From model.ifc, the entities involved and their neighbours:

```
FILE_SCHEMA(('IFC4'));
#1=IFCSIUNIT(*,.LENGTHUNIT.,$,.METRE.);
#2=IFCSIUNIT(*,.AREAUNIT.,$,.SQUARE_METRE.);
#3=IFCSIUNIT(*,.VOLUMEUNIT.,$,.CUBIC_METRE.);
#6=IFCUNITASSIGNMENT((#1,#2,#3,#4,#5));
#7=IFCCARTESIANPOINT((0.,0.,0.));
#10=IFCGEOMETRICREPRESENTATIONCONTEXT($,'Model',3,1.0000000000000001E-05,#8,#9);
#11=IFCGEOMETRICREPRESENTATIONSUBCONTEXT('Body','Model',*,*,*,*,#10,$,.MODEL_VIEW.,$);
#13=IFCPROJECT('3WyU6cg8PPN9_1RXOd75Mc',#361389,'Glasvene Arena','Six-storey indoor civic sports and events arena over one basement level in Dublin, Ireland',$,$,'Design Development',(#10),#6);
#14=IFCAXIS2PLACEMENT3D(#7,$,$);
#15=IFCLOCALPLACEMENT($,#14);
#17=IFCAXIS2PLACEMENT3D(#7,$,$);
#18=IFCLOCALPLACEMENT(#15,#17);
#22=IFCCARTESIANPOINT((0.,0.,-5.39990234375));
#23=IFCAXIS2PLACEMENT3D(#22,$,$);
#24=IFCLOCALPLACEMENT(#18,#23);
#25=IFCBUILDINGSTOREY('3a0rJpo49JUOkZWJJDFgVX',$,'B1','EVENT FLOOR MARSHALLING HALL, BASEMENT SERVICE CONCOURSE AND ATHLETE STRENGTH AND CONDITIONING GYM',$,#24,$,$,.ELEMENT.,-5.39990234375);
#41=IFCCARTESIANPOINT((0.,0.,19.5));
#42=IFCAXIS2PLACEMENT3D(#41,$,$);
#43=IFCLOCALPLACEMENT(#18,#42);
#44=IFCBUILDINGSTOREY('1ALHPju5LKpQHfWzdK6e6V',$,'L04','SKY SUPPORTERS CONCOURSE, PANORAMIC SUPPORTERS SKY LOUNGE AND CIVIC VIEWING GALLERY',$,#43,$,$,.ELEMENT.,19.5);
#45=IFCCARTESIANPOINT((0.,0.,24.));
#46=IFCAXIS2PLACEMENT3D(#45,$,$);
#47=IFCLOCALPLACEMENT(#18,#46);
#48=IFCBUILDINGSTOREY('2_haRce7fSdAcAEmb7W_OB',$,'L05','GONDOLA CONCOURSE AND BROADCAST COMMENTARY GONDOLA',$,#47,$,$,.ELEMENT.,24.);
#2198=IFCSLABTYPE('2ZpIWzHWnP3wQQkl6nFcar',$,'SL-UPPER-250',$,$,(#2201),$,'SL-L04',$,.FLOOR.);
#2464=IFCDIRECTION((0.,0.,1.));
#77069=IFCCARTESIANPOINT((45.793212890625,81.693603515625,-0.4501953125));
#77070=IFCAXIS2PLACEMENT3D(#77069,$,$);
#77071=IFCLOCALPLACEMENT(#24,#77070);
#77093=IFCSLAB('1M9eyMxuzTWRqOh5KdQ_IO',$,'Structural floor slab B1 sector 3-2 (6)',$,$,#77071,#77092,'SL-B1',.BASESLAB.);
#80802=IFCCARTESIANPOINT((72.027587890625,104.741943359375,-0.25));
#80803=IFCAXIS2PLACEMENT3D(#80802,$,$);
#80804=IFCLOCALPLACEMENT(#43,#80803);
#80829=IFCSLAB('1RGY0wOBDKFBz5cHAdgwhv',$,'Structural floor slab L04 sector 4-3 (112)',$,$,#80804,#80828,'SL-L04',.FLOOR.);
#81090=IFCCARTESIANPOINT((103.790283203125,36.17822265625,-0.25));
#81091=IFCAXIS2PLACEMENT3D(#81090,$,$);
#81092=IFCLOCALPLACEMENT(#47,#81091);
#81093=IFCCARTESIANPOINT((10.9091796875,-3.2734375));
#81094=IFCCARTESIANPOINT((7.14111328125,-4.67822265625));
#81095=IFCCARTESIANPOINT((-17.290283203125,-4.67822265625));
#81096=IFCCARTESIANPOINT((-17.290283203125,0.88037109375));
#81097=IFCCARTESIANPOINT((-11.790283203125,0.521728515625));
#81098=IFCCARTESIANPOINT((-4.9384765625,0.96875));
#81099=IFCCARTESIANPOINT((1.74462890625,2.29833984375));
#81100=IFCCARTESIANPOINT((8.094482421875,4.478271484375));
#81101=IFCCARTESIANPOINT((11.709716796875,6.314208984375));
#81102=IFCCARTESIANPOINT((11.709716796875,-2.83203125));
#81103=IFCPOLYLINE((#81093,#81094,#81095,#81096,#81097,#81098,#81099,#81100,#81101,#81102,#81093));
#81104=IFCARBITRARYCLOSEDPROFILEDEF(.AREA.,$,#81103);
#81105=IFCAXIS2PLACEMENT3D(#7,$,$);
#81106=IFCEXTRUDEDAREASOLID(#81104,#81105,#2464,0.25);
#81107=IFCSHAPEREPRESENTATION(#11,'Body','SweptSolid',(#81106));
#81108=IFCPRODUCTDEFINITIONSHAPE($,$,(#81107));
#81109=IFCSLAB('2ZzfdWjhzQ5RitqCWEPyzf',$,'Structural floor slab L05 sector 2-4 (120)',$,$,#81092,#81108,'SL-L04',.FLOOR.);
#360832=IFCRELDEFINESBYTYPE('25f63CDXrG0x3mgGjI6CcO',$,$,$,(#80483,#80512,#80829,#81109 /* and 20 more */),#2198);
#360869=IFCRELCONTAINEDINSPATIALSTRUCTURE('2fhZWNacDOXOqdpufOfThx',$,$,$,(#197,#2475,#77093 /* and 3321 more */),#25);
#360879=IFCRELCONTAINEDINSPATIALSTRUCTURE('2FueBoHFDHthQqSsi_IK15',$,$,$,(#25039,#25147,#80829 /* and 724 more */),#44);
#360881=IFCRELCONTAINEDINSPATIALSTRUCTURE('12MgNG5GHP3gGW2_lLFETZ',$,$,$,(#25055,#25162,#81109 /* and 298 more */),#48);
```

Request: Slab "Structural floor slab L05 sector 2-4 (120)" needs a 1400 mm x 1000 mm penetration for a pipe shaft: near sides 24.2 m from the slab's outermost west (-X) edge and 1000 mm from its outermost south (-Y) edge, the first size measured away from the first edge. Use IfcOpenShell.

```python
import numpy as np
import ifcopenshell
import ifcopenshell.api.feature
import ifcopenshell.api.geometry
import ifcopenshell.api.root
import ifcopenshell.geom
import ifcopenshell.util.placement
import ifcopenshell.util.representation
import ifcopenshell.util.shape
import ifcopenshell.util.unit

model = ifcopenshell.open("model.ifc")
unit_scale = ifcopenshell.util.unit.calculate_unit_scale(model)
settings = ifcopenshell.geom.settings()


def volume(element):
    """Net volume in cubic metres, openings subtracted."""
    shape = ifcopenshell.geom.create_shape(settings, element)
    return ifcopenshell.util.shape.get_volume(shape.geometry)


slab = model.by_guid("2ZzfdWjhzQ5RitqCWEPyzf")
before = volume(slab)

# Extent in the slab's own axes, in metres. The edges named are its -X and -Y sides.
slab_shape = ifcopenshell.geom.create_shape(settings, slab)
vertices = ifcopenshell.util.shape.get_vertices(slab_shape.geometry)
x_min, y_min, bottom = vertices.min(axis=0)
top = vertices[:, 2].max()

opening = ifcopenshell.api.root.create_entity(model, ifc_class="IfcOpeningElement", name="Pipe shaft opening", predefined_type="OPENING")
context = ifcopenshell.util.representation.get_context(model, "Model", "Body", "MODEL_VIEW")
width, depth = 1.4, 1
outline = [(0.0, 0.0), (width, 0.0), (width, depth), (0.0, depth), (0.0, 0.0)]
# Overshoot both faces by 50 mm so the cut is clean.
shape = ifcopenshell.api.geometry.add_slab_representation(
    model, context=context, depth=top - bottom + 0.1, polyline=outline
)
ifcopenshell.api.geometry.assign_representation(model, product=opening, representation=shape)

matrix = ifcopenshell.util.placement.get_local_placement(slab.ObjectPlacement)
matrix[:, 3] = matrix @ np.append(np.array([x_min + 24.2, y_min + 1, bottom - 0.05]) / unit_scale, 1.0)
ifcopenshell.api.geometry.edit_object_placement(model, product=opening, matrix=matrix, is_si=False)
ifcopenshell.api.feature.add_feature(model, feature=opening, element=slab)

after = volume(slab)

print(f"slab volume {before:.3f} -> {after:.3f} m3")

model.write("model_v2.ifc")
```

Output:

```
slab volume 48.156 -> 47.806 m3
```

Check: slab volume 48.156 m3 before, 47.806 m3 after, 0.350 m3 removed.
